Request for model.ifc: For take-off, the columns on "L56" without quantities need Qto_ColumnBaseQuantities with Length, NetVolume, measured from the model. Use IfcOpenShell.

First a look at what the model holds.

```python
import ifcopenshell
import ifcopenshell.util.element
import ifcopenshell.util.unit

model = ifcopenshell.open("model.ifc")
print(model.schema)
for unit_type in ("LENGTHUNIT", "AREAUNIT", "VOLUMEUNIT"):
    print(unit_type, ifcopenshell.util.unit.calculate_unit_scale(model, unit_type))
storey = next(s for s in model.by_type("IfcBuildingStorey") if s.Name == "L56")
columns = [e for e in ifcopenshell.util.element.get_decomposition(storey) if e.is_a("IfcColumn")]
for e in sorted(columns, key=lambda e: e.id()):
    print(e.id(), e.is_a(), e.Name, list(ifcopenshell.util.element.get_psets(e, qtos_only=True)), sep=" | ")
```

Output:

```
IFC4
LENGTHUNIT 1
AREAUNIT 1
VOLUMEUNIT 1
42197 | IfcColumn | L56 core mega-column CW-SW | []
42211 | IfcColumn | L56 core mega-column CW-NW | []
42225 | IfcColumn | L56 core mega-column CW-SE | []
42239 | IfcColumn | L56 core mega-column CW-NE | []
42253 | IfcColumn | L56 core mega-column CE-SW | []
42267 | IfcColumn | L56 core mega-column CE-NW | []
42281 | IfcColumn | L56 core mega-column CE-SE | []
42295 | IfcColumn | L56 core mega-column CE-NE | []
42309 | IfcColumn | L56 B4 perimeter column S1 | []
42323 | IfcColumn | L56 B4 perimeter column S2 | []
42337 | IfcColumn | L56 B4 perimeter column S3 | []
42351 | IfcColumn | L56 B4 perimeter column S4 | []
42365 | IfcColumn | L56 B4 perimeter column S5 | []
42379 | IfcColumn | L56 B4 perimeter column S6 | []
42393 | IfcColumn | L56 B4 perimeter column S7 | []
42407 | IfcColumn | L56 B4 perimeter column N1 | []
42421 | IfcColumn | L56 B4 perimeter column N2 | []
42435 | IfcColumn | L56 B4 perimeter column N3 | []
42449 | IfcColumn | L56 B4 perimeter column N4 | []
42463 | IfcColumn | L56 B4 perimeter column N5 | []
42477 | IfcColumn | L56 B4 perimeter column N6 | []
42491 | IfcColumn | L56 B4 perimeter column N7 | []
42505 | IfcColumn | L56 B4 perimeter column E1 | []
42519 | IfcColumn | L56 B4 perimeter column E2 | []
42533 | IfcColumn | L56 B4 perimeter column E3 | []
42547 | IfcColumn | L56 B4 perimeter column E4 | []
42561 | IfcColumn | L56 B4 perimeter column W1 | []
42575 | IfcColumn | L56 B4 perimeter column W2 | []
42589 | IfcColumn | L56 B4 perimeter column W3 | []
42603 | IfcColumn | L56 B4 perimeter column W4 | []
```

```python
import ifcopenshell
import ifcopenshell.api.pset
import ifcopenshell.geom
import ifcopenshell.util.element
import ifcopenshell.util.shape
import ifcopenshell.util.unit

model = ifcopenshell.open("model.ifc")
unit_scale = ifcopenshell.util.unit.calculate_unit_scale(model)
volume_scale = ifcopenshell.util.unit.calculate_unit_scale(model, "VOLUMEUNIT")
settings = ifcopenshell.geom.settings()

storey = next(s for s in model.by_type("IfcBuildingStorey") if s.Name == "L56")
columns = [e for e in ifcopenshell.util.element.get_decomposition(storey) if e.is_a("IfcColumn")]

for e in sorted(columns, key=lambda e: e.id()):
    if ifcopenshell.util.element.get_psets(e, qtos_only=True, should_inherit=False):
        continue
    # Geometry comes back in metres, in the element's own axes.
    shape = ifcopenshell.geom.create_shape(settings, e)
    values = {
        "Length": ifcopenshell.util.shape.get_z(shape.geometry) / unit_scale,
        "NetVolume": ifcopenshell.util.shape.get_volume(shape.geometry) / volume_scale,
    }
    qto = ifcopenshell.api.pset.add_qto(model, product=e, name="Qto_ColumnBaseQuantities")
    ifcopenshell.api.pset.edit_qto(model, qto=qto, properties=values)
    print(e.id(), {k: round(v, 3) for k, v in values.items()})

model.write("model_v2.ifc")
```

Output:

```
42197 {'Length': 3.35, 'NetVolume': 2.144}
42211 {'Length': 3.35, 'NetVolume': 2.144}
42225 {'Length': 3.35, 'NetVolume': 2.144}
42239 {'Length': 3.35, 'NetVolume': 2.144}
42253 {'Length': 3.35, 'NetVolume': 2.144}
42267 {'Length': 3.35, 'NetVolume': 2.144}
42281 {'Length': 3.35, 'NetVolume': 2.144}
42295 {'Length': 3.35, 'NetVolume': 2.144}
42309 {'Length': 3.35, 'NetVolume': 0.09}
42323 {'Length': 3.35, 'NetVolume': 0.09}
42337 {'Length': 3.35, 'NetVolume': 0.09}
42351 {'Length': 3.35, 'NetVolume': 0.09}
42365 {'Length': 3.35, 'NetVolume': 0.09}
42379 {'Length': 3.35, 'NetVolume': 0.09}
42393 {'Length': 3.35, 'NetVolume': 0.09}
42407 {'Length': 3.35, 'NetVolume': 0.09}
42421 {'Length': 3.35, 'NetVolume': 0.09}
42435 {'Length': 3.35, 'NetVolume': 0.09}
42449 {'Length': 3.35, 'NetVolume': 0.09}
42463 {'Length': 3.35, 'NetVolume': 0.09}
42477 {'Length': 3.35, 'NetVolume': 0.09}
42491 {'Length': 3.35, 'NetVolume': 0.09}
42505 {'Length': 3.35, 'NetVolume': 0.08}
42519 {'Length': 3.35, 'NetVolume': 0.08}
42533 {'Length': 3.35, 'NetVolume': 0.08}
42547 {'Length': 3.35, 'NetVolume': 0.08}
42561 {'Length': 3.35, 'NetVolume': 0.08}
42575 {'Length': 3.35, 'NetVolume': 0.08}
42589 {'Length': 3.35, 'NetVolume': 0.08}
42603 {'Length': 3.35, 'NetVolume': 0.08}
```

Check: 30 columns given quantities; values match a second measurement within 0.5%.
